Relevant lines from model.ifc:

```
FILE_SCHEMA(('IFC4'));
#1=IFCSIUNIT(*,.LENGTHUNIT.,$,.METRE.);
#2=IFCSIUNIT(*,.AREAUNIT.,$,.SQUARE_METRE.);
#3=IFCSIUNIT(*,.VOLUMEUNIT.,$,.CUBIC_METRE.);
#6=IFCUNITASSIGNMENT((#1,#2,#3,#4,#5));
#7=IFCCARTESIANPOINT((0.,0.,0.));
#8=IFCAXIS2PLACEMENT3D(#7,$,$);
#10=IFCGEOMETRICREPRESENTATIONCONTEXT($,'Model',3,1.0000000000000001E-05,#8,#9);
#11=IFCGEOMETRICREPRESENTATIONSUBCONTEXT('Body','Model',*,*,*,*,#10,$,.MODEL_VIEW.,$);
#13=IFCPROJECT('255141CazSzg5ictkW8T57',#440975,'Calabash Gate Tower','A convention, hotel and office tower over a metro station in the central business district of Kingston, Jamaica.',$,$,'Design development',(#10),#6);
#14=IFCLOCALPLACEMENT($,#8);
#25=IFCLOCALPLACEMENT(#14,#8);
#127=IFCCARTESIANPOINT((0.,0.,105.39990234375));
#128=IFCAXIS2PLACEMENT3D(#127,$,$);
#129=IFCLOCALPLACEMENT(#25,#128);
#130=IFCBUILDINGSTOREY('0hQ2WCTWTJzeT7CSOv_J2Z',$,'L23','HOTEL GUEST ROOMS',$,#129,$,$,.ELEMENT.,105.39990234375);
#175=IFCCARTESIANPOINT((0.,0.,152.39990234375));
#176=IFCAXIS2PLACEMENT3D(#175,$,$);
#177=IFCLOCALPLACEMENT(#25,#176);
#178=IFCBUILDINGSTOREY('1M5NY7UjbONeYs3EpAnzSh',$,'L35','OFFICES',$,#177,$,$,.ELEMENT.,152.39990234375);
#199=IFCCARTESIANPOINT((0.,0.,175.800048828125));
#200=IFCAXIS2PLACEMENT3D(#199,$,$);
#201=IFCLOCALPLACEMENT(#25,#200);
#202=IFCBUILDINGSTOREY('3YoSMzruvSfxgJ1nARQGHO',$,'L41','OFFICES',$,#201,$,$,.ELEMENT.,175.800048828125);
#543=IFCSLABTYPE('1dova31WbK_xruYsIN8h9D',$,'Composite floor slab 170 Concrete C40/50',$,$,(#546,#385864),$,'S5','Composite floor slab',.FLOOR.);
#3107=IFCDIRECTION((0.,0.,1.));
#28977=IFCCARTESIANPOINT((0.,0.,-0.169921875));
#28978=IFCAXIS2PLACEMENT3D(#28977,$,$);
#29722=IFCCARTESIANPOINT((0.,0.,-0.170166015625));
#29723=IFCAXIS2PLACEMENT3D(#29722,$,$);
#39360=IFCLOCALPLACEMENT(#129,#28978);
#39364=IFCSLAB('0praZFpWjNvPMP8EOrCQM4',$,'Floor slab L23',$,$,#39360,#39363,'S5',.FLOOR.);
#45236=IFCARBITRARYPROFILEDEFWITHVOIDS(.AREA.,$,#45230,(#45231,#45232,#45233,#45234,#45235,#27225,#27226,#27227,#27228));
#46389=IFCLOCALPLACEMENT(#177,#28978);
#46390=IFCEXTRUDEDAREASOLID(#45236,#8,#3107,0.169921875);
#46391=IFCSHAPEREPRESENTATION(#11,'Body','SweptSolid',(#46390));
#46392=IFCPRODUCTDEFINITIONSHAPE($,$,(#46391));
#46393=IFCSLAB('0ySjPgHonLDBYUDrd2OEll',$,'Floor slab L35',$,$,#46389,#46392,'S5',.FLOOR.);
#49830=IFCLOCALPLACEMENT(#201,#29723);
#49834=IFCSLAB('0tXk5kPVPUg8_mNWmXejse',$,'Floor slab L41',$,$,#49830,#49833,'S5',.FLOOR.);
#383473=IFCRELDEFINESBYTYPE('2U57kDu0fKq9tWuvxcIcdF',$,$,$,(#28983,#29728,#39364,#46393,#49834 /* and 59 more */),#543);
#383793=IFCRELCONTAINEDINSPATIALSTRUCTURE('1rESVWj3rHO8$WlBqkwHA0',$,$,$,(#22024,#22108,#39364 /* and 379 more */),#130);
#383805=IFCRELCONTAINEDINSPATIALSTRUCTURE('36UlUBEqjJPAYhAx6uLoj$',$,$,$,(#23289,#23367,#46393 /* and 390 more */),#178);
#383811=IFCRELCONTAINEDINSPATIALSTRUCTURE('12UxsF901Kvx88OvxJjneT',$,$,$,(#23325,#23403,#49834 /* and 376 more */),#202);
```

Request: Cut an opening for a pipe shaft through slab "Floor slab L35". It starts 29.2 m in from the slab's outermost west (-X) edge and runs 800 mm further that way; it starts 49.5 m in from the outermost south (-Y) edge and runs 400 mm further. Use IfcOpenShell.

```python
import numpy as np
import ifcopenshell
import ifcopenshell.api.feature
import ifcopenshell.api.geometry
import ifcopenshell.api.root
import ifcopenshell.geom
import ifcopenshell.util.placement
import ifcopenshell.util.representation
import ifcopenshell.util.shape
import ifcopenshell.util.unit

model = ifcopenshell.open("model.ifc")
unit_scale = ifcopenshell.util.unit.calculate_unit_scale(model)
settings = ifcopenshell.geom.settings()


def volume(element):
    """Net volume in cubic metres, openings subtracted."""
    shape = ifcopenshell.geom.create_shape(settings, element)
    return ifcopenshell.util.shape.get_volume(shape.geometry)


slab = model.by_id(46393)
before = volume(slab)

# Extent in the slab's own axes, in metres. The edges named are its -X and -Y sides.
slab_shape = ifcopenshell.geom.create_shape(settings, slab)
vertices = ifcopenshell.util.shape.get_vertices(slab_shape.geometry)
x_min, y_min, bottom = vertices.min(axis=0)
top = vertices[:, 2].max()

opening = ifcopenshell.api.root.create_entity(model, ifc_class="IfcOpeningElement", name="Pipe shaft opening", predefined_type="OPENING")
context = ifcopenshell.util.representation.get_context(model, "Model", "Body", "MODEL_VIEW")
width, depth = 0.8, 0.4
outline = [(0.0, 0.0), (width, 0.0), (width, depth), (0.0, depth), (0.0, 0.0)]
# Overshoot both faces by 50 mm so the cut is clean.
shape = ifcopenshell.api.geometry.add_slab_representation(
    model, context=context, depth=top - bottom + 0.1, polyline=outline
)
ifcopenshell.api.geometry.assign_representation(model, product=opening, representation=shape)

matrix = ifcopenshell.util.placement.get_local_placement(slab.ObjectPlacement)
matrix[:, 3] = matrix @ np.append(np.array([x_min + 29.2, y_min + 49.5, bottom - 0.05]) / unit_scale, 1.0)
ifcopenshell.api.geometry.edit_object_placement(model, product=opening, matrix=matrix, is_si=False)
ifcopenshell.api.feature.add_feature(model, feature=opening, element=slab)

after = volume(slab)

print(f"slab volume {before:.3f} -> {after:.3f} m3")

model.write("model-out.ifc")
```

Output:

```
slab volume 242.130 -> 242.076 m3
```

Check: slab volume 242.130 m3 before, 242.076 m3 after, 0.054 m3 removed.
